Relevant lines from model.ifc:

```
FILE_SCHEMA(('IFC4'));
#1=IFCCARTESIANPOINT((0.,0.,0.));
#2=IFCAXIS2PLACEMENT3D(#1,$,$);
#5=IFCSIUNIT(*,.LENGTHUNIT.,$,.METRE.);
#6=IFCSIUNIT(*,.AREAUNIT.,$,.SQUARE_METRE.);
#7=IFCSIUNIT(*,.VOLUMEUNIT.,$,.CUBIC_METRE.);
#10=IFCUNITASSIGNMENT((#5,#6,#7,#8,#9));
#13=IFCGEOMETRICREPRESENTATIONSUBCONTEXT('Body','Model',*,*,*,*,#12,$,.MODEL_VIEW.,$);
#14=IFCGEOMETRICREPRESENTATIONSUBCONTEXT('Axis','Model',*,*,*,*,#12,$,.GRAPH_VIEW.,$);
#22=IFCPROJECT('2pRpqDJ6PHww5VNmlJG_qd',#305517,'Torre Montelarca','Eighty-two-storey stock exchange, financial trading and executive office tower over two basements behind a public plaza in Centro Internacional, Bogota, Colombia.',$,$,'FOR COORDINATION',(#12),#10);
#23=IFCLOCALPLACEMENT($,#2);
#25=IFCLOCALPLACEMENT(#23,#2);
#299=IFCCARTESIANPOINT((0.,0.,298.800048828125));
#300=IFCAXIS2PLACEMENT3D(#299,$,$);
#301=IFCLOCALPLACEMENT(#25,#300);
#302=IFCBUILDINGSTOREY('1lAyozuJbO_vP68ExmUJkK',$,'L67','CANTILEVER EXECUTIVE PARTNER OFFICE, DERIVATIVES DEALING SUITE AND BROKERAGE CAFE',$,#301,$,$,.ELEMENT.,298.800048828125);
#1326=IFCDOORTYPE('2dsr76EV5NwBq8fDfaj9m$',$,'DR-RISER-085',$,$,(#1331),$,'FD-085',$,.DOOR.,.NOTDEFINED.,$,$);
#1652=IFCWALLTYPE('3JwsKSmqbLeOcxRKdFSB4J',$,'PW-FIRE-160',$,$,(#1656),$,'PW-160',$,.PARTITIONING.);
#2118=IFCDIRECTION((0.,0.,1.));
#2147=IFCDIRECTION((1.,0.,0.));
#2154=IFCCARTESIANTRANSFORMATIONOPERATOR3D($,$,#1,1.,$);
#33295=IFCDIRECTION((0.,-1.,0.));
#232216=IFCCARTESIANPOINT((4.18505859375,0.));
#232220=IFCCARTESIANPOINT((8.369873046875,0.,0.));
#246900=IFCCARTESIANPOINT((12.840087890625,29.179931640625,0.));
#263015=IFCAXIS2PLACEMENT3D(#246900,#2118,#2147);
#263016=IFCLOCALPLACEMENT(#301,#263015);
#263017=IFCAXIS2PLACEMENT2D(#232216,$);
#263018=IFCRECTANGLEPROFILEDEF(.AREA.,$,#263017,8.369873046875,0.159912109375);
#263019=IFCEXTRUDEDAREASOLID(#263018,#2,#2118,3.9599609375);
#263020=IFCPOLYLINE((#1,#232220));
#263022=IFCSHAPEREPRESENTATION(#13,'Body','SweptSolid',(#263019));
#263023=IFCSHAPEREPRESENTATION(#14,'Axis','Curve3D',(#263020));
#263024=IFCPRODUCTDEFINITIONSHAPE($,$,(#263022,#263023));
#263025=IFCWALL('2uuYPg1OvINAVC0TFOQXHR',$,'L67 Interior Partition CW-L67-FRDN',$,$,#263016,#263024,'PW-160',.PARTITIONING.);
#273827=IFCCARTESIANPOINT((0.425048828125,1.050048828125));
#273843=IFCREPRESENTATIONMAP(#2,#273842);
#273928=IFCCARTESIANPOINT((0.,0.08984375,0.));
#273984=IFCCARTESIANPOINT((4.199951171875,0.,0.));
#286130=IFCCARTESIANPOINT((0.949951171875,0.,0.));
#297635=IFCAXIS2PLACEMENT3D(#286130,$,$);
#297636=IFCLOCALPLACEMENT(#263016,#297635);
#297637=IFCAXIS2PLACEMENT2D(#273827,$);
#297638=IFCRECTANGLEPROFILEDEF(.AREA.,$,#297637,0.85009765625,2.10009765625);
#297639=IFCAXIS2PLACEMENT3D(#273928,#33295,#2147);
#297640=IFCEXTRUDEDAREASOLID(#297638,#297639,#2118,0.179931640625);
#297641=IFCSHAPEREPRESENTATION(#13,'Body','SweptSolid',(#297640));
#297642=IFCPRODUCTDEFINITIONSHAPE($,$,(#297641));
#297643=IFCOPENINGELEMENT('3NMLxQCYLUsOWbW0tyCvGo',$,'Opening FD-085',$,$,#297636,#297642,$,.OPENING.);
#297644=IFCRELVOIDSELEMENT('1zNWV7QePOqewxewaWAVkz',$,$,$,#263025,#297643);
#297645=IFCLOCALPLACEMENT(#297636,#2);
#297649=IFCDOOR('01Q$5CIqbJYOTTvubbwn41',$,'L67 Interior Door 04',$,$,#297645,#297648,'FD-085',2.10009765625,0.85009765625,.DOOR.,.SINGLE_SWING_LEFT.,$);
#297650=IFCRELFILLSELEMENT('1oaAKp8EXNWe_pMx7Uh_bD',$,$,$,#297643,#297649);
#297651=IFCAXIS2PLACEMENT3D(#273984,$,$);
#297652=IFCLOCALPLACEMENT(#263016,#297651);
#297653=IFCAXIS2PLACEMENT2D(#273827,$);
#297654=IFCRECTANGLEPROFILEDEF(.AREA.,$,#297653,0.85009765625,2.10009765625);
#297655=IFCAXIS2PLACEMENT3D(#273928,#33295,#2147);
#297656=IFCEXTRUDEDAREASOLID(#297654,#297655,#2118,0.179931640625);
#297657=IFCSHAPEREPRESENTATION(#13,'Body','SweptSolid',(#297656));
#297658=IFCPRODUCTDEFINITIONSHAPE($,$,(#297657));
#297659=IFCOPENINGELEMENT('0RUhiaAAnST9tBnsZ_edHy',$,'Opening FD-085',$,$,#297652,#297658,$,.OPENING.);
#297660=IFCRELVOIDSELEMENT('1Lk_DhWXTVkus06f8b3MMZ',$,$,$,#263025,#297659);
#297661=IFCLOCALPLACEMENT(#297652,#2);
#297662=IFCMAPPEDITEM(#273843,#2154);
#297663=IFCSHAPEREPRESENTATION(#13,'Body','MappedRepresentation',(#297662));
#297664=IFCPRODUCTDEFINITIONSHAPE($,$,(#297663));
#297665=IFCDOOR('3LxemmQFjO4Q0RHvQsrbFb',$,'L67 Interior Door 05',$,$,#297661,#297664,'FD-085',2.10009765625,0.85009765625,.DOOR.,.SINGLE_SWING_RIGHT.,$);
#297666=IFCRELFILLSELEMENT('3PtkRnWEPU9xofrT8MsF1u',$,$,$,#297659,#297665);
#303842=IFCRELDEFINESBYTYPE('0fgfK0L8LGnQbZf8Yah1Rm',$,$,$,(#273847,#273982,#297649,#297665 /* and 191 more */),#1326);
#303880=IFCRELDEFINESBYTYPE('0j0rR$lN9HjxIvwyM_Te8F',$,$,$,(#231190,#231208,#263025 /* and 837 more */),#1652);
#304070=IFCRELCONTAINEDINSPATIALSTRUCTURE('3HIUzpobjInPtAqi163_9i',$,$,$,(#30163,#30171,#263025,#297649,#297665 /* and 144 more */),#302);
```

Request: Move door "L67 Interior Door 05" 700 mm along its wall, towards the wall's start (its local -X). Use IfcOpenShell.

```python
import ifcopenshell
import ifcopenshell.api.geometry
import ifcopenshell.util.placement
import ifcopenshell.util.unit

model = ifcopenshell.open("model.ifc")
unit_scale = ifcopenshell.util.unit.calculate_unit_scale(model)

door = model.by_id(297665)
opening = door.FillsVoids[0].RelatingOpeningElement
wall = opening.VoidsElements[0].RelatingBuildingElement

wall_matrix = ifcopenshell.util.placement.get_local_placement(wall.ObjectPlacement)
shift = wall_matrix[:3, 0] * -0.7 / unit_scale
before = ifcopenshell.util.placement.get_local_placement(door.ObjectPlacement)[:3, 3].copy()

# The door is placed relative to its opening, so it follows when the opening moves.
matrix = ifcopenshell.util.placement.get_local_placement(opening.ObjectPlacement)
matrix[:3, 3] += shift
ifcopenshell.api.geometry.edit_object_placement(
    model, product=opening, matrix=matrix, is_si=False, should_transform_children=True
)

after = ifcopenshell.util.placement.get_local_placement(door.ObjectPlacement)[:3, 3]
print("door moved by", (after - before).round(3) + 0.0)

model.write("model_edited.ifc")
```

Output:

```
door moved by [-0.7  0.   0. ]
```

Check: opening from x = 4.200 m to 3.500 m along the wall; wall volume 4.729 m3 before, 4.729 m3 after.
